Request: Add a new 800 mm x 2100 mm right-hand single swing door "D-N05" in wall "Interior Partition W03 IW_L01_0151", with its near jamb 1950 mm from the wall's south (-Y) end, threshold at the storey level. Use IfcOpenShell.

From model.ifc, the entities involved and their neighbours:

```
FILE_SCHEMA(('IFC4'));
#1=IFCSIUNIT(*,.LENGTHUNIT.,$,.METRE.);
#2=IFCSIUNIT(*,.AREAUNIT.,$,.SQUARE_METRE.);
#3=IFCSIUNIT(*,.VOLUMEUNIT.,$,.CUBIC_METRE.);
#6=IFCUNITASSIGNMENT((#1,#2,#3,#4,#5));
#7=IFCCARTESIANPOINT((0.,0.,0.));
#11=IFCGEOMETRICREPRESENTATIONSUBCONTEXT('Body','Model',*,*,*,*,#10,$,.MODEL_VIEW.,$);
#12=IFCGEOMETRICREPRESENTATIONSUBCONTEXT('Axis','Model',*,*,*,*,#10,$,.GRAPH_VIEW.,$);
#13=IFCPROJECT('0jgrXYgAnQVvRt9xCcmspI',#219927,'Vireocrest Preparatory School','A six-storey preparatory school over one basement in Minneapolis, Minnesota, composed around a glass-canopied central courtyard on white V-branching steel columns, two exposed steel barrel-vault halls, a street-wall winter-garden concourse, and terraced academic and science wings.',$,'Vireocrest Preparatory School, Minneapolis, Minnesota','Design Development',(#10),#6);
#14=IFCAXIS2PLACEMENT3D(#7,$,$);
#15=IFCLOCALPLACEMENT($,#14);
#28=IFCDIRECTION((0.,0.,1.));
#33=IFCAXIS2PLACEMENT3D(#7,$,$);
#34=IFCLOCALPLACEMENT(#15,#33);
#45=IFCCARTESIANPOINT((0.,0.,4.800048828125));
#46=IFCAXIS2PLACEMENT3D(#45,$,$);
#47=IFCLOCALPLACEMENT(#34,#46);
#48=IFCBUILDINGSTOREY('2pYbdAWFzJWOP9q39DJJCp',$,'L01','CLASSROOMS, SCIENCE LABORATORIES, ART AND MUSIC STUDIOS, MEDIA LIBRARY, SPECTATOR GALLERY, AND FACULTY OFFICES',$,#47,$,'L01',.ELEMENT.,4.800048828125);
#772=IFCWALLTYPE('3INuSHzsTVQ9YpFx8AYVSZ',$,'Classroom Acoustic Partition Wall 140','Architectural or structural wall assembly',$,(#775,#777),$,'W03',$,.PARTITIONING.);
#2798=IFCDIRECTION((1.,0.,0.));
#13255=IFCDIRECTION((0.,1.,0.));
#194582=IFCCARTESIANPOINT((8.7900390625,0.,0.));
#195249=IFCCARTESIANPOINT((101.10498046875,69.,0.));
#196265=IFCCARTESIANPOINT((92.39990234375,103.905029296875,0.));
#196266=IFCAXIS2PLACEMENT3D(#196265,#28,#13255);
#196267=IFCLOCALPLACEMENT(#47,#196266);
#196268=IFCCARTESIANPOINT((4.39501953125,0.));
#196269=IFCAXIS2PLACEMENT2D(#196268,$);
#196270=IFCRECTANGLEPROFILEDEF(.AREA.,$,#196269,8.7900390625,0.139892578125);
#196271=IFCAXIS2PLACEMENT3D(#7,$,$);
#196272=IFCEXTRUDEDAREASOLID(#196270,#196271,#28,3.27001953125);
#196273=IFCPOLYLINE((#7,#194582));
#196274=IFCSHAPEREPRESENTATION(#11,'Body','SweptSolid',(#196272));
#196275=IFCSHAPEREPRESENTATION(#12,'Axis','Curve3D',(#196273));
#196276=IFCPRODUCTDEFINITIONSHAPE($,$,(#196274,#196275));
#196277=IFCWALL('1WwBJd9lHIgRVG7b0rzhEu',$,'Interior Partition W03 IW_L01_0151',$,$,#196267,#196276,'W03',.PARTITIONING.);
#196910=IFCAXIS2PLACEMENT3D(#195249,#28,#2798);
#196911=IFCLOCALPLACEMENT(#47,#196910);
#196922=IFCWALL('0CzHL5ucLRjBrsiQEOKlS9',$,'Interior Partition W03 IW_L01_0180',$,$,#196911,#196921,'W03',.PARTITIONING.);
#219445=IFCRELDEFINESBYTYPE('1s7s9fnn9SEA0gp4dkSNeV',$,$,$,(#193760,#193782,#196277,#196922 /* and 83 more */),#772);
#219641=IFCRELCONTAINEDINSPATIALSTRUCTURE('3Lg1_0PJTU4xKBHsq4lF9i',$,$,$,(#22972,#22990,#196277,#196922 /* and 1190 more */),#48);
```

```python
import numpy as np
import ifcopenshell
import ifcopenshell.api.feature
import ifcopenshell.api.geometry
import ifcopenshell.api.root
import ifcopenshell.api.spatial
import ifcopenshell.geom
import ifcopenshell.util.element
import ifcopenshell.util.placement
import ifcopenshell.util.representation
import ifcopenshell.util.shape
import ifcopenshell.util.unit

model = ifcopenshell.open("model.ifc")
unit_scale = ifcopenshell.util.unit.calculate_unit_scale(model)
settings = ifcopenshell.geom.settings()


def volume(element):
    """Net volume in cubic metres, openings subtracted."""
    shape = ifcopenshell.geom.create_shape(settings, element)
    return ifcopenshell.util.shape.get_volume(shape.geometry)


wall = model.by_guid("1WwBJd9lHIgRVG7b0rzhEu")
storey = ifcopenshell.util.element.get_container(wall, ifc_class="IfcBuildingStorey")
context = ifcopenshell.util.representation.get_context(model, "Model", "Body", "MODEL_VIEW")
before = volume(wall)

width, height, from_end, sill = 0.8, 2.1, 1.95, 0.0  # metres

# The wall runs along its own X axis, and the end named is its -X end.
wall_shape = ifcopenshell.geom.create_shape(settings, wall)
x, y, z = ifcopenshell.util.shape.get_vertices(wall_shape.geometry).T
start = x.min() + from_end
face, thickness = float(y.min()), float(y.max() - y.min())
wall_matrix = ifcopenshell.util.placement.get_local_placement(wall.ObjectPlacement)
level = ifcopenshell.util.placement.get_local_placement(storey.ObjectPlacement)[2, 3]


def in_wall(x, y):
    """Placement at x, y metres in the wall's axes, at sill height."""
    matrix = wall_matrix.copy()
    matrix[:, 3] = wall_matrix @ np.array([x / unit_scale, y / unit_scale, 0.0, 1.0])
    matrix[2, 3] = level + sill / unit_scale
    return matrix


# Opening: a box that overshoots both wall faces by 50 mm.
opening = ifcopenshell.api.root.create_entity(model, ifc_class="IfcOpeningElement", predefined_type="OPENING")
box = ifcopenshell.api.geometry.add_wall_representation(
    model, context=context, length=width, height=height, thickness=thickness + 0.1
)
ifcopenshell.api.geometry.assign_representation(model, product=opening, representation=box)
ifcopenshell.api.geometry.edit_object_placement(model, product=opening, matrix=in_wall(start, face - 0.05), is_si=False)
ifcopenshell.api.feature.add_feature(model, feature=opening, element=wall)

door = ifcopenshell.api.root.create_entity(model, ifc_class="IfcDoor", name="D-N05", predefined_type="DOOR")
door.OverallWidth, door.OverallHeight = width / unit_scale, height / unit_scale
door.OperationType = "SINGLE_SWING_RIGHT"
body = ifcopenshell.api.geometry.add_door_representation(
    model,
    context=context,
    overall_width=door.OverallWidth,
    overall_height=door.OverallHeight,
    operation_type="SINGLE_SWING_RIGHT",
    lining_properties={"LiningDepth": thickness / unit_scale, "ThresholdDepth": thickness / unit_scale},
)
ifcopenshell.api.geometry.assign_representation(model, product=door, representation=body)
ifcopenshell.api.spatial.assign_container(model, products=[door], relating_structure=storey)
ifcopenshell.api.feature.add_filling(model, opening=opening, element=door)

# The lining spans the wall, so the door starts at the wall face.
ifcopenshell.api.geometry.edit_object_placement(model, product=door, matrix=in_wall(start, face), is_si=False)

after = volume(wall)

print(f"wall volume {before:.3f} -> {after:.3f} m3")

model.write("model_v2.ifc")
```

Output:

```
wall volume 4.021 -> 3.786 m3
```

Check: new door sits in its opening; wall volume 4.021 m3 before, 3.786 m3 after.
